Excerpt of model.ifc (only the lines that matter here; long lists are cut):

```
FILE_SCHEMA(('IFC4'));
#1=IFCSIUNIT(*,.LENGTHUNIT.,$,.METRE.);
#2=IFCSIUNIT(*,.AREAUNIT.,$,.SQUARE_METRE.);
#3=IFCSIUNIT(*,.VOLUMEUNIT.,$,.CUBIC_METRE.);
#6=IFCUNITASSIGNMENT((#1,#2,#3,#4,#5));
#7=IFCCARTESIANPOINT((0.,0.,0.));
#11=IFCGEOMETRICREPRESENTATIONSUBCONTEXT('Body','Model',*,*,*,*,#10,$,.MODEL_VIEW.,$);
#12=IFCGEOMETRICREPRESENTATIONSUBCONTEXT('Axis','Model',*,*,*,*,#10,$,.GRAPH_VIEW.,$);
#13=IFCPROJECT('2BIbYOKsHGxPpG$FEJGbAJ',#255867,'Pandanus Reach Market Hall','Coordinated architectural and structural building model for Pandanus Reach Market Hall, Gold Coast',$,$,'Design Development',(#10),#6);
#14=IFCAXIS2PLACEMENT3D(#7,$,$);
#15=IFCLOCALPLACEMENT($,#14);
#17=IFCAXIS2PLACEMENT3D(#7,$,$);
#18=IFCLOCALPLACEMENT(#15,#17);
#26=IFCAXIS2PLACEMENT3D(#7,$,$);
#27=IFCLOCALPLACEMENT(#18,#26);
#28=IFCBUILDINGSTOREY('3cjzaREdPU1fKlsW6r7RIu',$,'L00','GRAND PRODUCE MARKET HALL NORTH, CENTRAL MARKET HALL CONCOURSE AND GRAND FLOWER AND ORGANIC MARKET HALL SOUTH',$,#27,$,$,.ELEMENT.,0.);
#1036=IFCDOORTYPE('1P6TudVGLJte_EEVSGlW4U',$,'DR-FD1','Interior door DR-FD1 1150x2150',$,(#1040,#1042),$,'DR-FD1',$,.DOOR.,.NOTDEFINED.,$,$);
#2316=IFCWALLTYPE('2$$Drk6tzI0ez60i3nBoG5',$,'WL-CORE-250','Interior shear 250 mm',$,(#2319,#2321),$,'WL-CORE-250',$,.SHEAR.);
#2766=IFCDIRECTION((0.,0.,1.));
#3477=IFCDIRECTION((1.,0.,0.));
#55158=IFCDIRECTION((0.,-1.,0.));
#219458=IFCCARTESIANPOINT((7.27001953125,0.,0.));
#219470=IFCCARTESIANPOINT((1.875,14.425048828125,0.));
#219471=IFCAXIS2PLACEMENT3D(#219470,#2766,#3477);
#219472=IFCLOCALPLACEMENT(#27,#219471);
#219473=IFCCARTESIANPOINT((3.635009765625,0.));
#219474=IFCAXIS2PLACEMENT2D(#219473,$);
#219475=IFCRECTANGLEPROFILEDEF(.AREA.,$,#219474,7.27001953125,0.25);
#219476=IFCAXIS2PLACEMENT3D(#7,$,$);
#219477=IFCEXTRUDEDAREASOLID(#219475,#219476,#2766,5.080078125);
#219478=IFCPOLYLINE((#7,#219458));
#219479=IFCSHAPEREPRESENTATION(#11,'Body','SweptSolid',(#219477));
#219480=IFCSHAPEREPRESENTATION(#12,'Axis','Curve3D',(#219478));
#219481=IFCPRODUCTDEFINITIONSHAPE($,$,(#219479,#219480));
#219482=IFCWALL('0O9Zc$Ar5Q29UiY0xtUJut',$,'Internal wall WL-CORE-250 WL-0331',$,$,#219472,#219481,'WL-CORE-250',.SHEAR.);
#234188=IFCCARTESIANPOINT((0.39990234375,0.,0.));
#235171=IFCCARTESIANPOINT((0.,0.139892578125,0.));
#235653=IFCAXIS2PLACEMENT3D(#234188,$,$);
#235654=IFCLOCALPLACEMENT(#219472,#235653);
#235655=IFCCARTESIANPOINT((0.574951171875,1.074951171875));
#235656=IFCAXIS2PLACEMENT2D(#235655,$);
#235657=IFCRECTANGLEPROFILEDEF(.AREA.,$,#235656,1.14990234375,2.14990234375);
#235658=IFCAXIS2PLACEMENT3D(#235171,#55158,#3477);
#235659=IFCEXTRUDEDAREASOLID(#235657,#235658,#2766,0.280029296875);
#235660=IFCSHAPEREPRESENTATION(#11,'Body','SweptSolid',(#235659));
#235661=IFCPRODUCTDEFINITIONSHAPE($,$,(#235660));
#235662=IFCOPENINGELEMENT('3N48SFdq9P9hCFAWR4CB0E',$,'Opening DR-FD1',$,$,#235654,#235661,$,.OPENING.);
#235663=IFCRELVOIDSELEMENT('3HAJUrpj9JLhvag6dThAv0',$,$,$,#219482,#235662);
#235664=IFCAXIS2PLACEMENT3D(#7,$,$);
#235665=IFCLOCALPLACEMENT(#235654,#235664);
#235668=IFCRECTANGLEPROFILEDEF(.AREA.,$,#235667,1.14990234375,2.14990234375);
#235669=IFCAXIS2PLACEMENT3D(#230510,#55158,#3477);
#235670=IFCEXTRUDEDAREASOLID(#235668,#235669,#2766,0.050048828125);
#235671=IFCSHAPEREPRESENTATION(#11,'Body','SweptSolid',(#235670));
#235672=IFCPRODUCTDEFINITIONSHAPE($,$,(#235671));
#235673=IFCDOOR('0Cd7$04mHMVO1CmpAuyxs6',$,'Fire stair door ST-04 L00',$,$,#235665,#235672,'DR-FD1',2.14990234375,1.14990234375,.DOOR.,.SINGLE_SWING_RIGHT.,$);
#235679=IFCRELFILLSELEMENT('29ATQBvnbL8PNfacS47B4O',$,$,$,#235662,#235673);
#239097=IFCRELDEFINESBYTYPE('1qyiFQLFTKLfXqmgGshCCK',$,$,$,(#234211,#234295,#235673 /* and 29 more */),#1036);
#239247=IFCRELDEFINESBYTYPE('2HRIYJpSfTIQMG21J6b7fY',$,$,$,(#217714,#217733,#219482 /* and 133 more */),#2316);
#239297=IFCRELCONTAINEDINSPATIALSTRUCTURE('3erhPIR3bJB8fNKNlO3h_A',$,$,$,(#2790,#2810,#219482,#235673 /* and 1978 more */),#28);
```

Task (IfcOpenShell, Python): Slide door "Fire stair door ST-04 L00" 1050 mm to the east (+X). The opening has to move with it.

```python
import ifcopenshell
import ifcopenshell.api.geometry
import ifcopenshell.util.placement
import ifcopenshell.util.unit

model = ifcopenshell.open("model.ifc")
unit_scale = ifcopenshell.util.unit.calculate_unit_scale(model)

door = model.by_id(235673)
opening = door.FillsVoids[0].RelatingOpeningElement
wall = opening.VoidsElements[0].RelatingBuildingElement

wall_matrix = ifcopenshell.util.placement.get_local_placement(wall.ObjectPlacement)
shift = wall_matrix[:3, 0] * 1.05 / unit_scale
before = ifcopenshell.util.placement.get_local_placement(door.ObjectPlacement)[:3, 3].copy()

# The door is placed relative to its opening, so it follows when the opening moves.
matrix = ifcopenshell.util.placement.get_local_placement(opening.ObjectPlacement)
matrix[:3, 3] += shift
ifcopenshell.api.geometry.edit_object_placement(
    model, product=opening, matrix=matrix, is_si=False, should_transform_children=True
)

after = ifcopenshell.util.placement.get_local_placement(door.ObjectPlacement)[:3, 3]
print("door moved by", (after - before).round(3) + 0.0)

model.write("model_rev.ifc")
```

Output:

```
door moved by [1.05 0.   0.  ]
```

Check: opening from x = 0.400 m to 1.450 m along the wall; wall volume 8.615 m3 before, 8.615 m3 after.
